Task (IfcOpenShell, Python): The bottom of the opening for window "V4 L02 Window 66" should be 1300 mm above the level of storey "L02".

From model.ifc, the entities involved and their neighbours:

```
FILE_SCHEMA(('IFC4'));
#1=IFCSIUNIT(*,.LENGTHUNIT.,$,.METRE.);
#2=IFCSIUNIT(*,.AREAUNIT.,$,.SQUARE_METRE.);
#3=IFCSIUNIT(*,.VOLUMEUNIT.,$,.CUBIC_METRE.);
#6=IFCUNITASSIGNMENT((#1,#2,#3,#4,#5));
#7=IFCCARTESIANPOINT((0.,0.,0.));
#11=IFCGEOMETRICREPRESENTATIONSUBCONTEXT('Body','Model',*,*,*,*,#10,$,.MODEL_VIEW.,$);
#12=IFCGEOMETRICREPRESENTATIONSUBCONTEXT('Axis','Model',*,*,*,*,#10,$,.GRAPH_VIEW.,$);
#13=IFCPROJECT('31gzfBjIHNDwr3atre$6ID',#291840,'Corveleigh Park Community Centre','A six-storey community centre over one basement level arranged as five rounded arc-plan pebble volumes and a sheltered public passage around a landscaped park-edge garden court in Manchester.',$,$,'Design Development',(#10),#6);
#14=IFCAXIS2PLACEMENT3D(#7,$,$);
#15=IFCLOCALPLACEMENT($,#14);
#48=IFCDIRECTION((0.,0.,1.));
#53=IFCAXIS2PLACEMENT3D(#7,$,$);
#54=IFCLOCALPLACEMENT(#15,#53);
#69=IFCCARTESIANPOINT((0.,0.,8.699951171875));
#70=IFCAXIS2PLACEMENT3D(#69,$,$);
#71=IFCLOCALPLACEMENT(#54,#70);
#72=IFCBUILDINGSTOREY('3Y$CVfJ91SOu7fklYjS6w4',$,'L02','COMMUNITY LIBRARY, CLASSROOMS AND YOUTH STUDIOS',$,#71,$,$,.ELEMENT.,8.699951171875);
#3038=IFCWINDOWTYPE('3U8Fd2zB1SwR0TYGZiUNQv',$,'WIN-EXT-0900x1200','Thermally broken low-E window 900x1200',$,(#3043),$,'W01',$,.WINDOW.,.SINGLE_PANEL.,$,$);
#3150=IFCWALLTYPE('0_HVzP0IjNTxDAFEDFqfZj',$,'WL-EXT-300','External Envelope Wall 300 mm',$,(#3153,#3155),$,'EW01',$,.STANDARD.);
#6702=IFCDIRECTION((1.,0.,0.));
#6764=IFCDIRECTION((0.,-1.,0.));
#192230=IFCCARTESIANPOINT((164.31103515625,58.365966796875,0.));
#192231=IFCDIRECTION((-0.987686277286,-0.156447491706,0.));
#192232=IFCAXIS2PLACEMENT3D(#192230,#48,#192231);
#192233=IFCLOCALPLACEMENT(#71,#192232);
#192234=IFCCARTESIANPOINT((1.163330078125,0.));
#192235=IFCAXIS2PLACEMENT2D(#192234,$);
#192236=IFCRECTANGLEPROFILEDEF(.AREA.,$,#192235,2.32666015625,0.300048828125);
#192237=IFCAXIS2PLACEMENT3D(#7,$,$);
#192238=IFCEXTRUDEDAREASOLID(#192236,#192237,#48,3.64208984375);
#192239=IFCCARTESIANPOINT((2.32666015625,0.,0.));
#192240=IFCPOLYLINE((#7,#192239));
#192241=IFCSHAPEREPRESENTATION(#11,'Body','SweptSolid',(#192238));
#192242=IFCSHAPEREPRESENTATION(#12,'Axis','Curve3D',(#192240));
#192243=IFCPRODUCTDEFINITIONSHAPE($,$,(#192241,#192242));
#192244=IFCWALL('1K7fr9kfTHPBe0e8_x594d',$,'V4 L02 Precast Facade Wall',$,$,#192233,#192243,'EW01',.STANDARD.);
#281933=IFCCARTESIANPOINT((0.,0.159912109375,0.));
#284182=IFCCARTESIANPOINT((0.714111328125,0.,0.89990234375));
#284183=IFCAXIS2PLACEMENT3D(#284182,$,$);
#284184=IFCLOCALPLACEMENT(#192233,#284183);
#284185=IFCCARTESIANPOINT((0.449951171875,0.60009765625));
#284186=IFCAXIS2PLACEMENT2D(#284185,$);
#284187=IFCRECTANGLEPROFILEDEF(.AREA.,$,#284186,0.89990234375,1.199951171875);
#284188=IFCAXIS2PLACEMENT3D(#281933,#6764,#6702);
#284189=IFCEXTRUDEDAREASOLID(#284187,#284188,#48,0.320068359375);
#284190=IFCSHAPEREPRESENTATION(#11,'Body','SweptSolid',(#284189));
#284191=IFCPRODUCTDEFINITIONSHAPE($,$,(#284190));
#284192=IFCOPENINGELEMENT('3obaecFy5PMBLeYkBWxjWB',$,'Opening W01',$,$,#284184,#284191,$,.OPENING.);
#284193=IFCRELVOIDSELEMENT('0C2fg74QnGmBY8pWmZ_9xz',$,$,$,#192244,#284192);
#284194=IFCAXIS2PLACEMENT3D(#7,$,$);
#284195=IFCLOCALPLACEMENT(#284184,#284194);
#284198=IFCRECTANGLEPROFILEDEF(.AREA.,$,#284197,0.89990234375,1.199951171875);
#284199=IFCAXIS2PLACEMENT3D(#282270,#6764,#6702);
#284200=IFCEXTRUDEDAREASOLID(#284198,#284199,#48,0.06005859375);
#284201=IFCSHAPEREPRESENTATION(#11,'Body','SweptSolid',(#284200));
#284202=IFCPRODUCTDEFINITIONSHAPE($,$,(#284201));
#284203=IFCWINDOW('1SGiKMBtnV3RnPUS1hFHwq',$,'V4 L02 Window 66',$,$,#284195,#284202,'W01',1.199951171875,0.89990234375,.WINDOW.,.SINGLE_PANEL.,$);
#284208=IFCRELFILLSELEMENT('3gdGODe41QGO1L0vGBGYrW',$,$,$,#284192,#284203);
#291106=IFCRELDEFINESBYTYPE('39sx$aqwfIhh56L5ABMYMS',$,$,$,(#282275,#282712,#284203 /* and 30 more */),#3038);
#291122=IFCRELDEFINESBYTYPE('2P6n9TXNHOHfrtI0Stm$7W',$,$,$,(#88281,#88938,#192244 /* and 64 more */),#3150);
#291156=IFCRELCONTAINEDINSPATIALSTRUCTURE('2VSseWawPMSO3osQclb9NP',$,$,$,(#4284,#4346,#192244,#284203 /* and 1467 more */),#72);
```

```python
import numpy as np
import ifcopenshell
import ifcopenshell.api.geometry
import ifcopenshell.geom
import ifcopenshell.util.element
import ifcopenshell.util.placement
import ifcopenshell.util.shape
import ifcopenshell.util.unit

model = ifcopenshell.open("model.ifc")
unit_scale = ifcopenshell.util.unit.calculate_unit_scale(model)

window = model.by_guid("1SGiKMBtnV3RnPUS1hFHwq")
opening = window.FillsVoids[0].RelatingOpeningElement
storey = ifcopenshell.util.element.get_container(window, ifc_class="IfcBuildingStorey")
level = ifcopenshell.util.placement.get_local_placement(storey.ObjectPlacement)[2, 3]

# The opening's origin need not be at the sill, so measure its lowest point.
shape = ifcopenshell.geom.create_shape(ifcopenshell.geom.settings(), opening)
bottom = ifcopenshell.util.shape.get_shape_bottom_elevation(shape, shape.geometry) / unit_scale
dz = level + 1.3 - bottom

shift = np.array([0.0, 0.0, dz])
# The window is placed relative to its opening, so it follows when the opening moves.
matrix = ifcopenshell.util.placement.get_local_placement(opening.ObjectPlacement)
matrix[:3, 3] += shift
ifcopenshell.api.geometry.edit_object_placement(
    model, product=opening, matrix=matrix, is_si=False, should_transform_children=True
)

print(f"moved by {dz * unit_scale:+.3f} m")

model.write("model-out.ifc")
```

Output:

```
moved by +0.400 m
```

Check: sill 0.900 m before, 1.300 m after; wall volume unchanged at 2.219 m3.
